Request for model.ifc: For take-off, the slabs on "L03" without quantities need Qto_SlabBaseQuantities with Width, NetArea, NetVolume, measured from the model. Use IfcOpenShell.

First a look at what the model holds.

```python
import ifcopenshell
import ifcopenshell.util.element
import ifcopenshell.util.unit

model = ifcopenshell.open("model.ifc")
print(model.schema)
for unit_type in ("LENGTHUNIT", "AREAUNIT", "VOLUMEUNIT"):
    print(unit_type, ifcopenshell.util.unit.calculate_unit_scale(model, unit_type))
storey = next(s for s in model.by_type("IfcBuildingStorey") if s.Name == "L03")
slabs = [e for e in ifcopenshell.util.element.get_decomposition(storey) if e.is_a("IfcSlab")]
for e in sorted(slabs, key=lambda e: e.id()):
    print(e.id(), e.is_a(), e.Name, list(ifcopenshell.util.element.get_psets(e, qtos_only=True)), sep=" | ")
```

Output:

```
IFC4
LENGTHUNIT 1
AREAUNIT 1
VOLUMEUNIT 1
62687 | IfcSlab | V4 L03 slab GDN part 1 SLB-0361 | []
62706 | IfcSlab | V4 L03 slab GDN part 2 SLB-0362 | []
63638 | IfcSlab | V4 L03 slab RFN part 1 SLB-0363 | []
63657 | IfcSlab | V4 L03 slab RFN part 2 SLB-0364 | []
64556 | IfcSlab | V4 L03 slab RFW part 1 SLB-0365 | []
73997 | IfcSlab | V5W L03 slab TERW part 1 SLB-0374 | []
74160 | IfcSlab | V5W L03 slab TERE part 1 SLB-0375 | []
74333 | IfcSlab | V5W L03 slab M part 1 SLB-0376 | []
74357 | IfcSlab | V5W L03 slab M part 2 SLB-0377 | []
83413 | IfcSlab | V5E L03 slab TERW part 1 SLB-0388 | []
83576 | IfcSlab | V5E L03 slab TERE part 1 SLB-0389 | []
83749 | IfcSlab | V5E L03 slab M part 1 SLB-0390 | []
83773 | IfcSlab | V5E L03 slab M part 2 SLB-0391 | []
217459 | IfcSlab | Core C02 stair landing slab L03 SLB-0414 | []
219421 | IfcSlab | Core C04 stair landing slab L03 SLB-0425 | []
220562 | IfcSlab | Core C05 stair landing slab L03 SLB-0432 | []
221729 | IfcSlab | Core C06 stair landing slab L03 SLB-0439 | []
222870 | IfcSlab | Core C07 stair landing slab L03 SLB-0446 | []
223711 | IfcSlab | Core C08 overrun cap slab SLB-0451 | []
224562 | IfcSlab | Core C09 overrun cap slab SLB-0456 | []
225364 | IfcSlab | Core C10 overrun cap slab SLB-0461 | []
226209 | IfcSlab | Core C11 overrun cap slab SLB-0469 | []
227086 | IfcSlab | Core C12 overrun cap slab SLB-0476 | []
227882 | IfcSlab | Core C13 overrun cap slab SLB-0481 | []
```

```python
import ifcopenshell
import ifcopenshell.api.pset
import ifcopenshell.geom
import ifcopenshell.util.element
import ifcopenshell.util.shape
import ifcopenshell.util.unit

model = ifcopenshell.open("model.ifc")
unit_scale = ifcopenshell.util.unit.calculate_unit_scale(model)
area_scale = ifcopenshell.util.unit.calculate_unit_scale(model, "AREAUNIT")
volume_scale = ifcopenshell.util.unit.calculate_unit_scale(model, "VOLUMEUNIT")
settings = ifcopenshell.geom.settings()

storey = next(s for s in model.by_type("IfcBuildingStorey") if s.Name == "L03")
slabs = [e for e in ifcopenshell.util.element.get_decomposition(storey) if e.is_a("IfcSlab")]

for e in sorted(slabs, key=lambda e: e.id()):
    if ifcopenshell.util.element.get_psets(e, qtos_only=True, should_inherit=False):
        continue
    # Geometry comes back in metres, in the element's own axes.
    shape = ifcopenshell.geom.create_shape(settings, e)
    values = {
        "Width": ifcopenshell.util.shape.get_z(shape.geometry) / unit_scale,
        "NetArea": ifcopenshell.util.shape.get_footprint_area(shape.geometry) / area_scale,
        "NetVolume": ifcopenshell.util.shape.get_volume(shape.geometry) / volume_scale,
    }
    qto = ifcopenshell.api.pset.add_qto(model, product=e, name="Qto_SlabBaseQuantities")
    ifcopenshell.api.pset.edit_qto(model, qto=qto, properties=values)
    print(e.id(), {k: round(v, 3) for k, v in values.items()})

model.write("model_edited.ifc")
```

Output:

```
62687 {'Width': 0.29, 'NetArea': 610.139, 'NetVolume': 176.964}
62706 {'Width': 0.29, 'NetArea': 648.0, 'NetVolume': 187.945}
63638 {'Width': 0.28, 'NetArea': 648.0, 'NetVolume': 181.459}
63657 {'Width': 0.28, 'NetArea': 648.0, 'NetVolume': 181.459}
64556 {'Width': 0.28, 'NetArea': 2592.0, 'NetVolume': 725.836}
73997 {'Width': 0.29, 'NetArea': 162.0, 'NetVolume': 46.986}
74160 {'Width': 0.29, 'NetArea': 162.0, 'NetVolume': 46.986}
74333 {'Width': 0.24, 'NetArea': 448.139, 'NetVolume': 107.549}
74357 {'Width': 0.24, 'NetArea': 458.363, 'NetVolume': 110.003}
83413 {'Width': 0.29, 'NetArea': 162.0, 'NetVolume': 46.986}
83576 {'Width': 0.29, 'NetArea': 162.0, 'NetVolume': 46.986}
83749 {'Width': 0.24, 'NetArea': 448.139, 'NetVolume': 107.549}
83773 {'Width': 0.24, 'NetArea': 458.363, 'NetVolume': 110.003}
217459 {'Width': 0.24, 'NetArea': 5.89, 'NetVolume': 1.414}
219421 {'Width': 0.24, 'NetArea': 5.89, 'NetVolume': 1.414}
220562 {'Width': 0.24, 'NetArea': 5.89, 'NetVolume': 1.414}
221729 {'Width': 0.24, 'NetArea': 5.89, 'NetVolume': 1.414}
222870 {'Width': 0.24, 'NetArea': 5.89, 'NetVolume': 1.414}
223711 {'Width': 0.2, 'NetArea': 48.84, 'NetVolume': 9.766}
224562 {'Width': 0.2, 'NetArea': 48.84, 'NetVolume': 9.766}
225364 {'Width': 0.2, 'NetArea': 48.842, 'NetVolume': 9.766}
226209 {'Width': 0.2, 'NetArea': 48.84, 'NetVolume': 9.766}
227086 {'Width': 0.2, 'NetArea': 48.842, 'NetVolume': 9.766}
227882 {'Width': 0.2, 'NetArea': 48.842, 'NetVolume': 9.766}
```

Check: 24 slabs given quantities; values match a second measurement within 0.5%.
